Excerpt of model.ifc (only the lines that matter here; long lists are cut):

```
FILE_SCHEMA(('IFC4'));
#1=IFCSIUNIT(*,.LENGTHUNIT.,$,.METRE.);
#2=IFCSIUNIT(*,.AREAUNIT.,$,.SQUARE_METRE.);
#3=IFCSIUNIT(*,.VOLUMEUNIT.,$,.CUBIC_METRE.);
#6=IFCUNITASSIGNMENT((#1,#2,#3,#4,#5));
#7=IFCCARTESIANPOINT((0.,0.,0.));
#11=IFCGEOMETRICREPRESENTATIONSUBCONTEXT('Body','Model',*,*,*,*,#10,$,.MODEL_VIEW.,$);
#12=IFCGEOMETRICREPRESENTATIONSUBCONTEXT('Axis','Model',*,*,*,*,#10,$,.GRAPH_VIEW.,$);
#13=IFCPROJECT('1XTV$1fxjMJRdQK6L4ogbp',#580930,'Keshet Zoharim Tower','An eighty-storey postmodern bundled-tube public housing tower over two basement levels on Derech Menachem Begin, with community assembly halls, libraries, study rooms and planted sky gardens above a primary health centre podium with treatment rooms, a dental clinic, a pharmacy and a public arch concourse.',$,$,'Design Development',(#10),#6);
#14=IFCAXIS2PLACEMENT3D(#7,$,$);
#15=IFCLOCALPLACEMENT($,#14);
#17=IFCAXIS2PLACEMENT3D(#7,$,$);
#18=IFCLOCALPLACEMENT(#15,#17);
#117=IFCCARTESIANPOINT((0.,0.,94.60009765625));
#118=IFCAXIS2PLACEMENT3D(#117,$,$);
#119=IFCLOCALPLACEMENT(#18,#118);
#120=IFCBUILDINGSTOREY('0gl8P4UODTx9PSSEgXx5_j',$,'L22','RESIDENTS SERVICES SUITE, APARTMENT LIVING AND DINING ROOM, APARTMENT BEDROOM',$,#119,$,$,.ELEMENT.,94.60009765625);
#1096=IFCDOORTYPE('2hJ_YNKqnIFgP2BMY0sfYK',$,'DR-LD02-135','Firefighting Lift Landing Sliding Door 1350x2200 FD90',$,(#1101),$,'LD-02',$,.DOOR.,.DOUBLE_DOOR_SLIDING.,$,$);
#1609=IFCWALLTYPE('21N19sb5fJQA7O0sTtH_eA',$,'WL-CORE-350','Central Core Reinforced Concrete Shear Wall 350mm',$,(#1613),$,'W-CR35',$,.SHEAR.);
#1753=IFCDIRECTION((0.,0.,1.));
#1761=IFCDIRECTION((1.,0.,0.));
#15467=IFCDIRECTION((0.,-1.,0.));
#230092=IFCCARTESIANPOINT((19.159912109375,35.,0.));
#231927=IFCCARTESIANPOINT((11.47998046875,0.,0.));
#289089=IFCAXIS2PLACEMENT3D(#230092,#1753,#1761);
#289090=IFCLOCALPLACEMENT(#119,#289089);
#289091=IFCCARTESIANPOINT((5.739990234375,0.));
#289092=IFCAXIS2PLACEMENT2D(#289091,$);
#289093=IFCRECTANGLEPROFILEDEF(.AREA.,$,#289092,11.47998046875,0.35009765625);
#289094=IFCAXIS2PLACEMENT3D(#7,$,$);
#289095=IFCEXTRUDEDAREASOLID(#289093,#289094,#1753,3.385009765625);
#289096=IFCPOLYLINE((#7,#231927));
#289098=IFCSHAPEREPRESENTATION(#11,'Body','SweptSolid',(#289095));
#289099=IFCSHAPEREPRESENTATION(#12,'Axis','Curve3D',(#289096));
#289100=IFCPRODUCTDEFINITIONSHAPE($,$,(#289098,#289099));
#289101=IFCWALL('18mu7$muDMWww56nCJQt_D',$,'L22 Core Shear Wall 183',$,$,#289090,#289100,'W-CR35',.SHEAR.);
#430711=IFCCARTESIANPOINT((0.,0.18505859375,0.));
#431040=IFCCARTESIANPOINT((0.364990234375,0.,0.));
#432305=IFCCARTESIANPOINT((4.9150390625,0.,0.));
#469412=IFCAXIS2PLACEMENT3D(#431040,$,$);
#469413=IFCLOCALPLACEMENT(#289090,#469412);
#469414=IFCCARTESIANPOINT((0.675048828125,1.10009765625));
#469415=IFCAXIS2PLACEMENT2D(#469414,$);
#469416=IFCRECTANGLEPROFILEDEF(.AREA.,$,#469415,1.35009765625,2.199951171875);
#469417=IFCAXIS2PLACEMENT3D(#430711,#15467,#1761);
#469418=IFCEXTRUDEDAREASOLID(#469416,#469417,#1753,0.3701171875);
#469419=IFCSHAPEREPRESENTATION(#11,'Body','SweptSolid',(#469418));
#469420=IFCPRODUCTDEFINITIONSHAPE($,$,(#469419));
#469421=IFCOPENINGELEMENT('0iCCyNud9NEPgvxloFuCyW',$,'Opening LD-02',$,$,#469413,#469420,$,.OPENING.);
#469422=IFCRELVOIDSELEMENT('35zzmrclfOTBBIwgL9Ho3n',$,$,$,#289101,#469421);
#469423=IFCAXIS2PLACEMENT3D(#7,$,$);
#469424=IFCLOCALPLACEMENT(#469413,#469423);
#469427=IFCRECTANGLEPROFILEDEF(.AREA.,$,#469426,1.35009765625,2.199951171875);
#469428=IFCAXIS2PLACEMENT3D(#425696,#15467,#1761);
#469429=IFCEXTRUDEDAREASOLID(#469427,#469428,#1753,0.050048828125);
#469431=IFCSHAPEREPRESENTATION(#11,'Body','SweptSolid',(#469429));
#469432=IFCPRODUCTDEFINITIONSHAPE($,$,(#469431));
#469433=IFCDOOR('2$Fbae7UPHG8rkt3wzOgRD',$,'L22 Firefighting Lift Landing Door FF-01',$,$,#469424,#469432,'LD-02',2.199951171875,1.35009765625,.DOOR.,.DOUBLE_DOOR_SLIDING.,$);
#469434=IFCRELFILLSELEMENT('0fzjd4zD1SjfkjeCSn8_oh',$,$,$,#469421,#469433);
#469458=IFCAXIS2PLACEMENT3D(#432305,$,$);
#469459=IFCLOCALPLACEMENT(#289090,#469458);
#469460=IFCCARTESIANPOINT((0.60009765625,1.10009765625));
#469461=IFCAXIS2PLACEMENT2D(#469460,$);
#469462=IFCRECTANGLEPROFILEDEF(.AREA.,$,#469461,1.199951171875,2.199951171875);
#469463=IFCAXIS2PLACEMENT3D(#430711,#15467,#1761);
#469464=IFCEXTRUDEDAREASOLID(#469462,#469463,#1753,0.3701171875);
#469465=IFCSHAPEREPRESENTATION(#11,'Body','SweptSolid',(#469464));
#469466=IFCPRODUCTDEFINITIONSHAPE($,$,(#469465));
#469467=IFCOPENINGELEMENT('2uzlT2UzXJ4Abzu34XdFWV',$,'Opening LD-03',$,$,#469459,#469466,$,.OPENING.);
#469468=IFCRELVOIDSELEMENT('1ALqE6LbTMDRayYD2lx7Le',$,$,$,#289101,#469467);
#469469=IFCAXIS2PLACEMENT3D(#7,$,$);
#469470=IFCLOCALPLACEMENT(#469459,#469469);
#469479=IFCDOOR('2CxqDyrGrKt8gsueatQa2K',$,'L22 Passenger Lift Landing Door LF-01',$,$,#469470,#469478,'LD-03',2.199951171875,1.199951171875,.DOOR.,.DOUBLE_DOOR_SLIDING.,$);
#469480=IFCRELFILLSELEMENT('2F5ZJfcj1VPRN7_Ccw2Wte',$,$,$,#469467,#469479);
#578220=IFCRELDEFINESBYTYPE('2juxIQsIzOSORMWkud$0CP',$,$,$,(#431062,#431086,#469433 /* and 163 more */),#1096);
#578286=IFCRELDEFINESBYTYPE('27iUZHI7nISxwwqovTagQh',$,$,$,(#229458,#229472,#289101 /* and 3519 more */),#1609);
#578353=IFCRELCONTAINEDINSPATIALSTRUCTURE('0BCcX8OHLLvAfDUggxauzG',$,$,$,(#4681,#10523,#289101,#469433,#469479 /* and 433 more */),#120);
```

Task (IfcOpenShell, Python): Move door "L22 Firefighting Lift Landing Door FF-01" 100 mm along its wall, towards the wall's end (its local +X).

```python
import ifcopenshell
import ifcopenshell.api.geometry
import ifcopenshell.util.placement
import ifcopenshell.util.unit

model = ifcopenshell.open("model.ifc")
unit_scale = ifcopenshell.util.unit.calculate_unit_scale(model)

door = model.by_guid("2$Fbae7UPHG8rkt3wzOgRD")
opening = door.FillsVoids[0].RelatingOpeningElement
wall = opening.VoidsElements[0].RelatingBuildingElement

wall_matrix = ifcopenshell.util.placement.get_local_placement(wall.ObjectPlacement)
shift = wall_matrix[:3, 0] * 0.1 / unit_scale
before = ifcopenshell.util.placement.get_local_placement(door.ObjectPlacement)[:3, 3].copy()

# The door is placed relative to its opening, so it follows when the opening moves.
matrix = ifcopenshell.util.placement.get_local_placement(opening.ObjectPlacement)
matrix[:3, 3] += shift
ifcopenshell.api.geometry.edit_object_placement(
    model, product=opening, matrix=matrix, is_si=False, should_transform_children=True
)

after = ifcopenshell.util.placement.get_local_placement(door.ObjectPlacement)[:3, 3]
print("door moved by", (after - before).round(3) + 0.0)

model.write("model_updated.ifc")
```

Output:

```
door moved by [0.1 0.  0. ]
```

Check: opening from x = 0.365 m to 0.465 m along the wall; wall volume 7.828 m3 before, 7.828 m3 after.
